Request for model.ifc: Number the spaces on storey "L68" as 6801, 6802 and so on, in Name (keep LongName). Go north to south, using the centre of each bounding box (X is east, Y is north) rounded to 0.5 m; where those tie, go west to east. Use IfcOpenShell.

First a look at what the model holds.

```python
import ifcopenshell
import ifcopenshell.util.element
import ifcopenshell.util.placement

model = ifcopenshell.open("model.ifc")
print(model.schema)
storey = next(s for s in model.by_type("IfcBuildingStorey") if s.Name == "L68")
spaces = [e for e in ifcopenshell.util.element.get_decomposition(storey) if e.is_a("IfcSpace")]
for e in sorted(spaces, key=lambda e: e.id()):
    origin = ifcopenshell.util.placement.get_local_placement(e.ObjectPlacement)[:3, 3]
    print(e.id(), e.Name, e.LongName, origin.round(2) + 0.0, sep=" | ")
```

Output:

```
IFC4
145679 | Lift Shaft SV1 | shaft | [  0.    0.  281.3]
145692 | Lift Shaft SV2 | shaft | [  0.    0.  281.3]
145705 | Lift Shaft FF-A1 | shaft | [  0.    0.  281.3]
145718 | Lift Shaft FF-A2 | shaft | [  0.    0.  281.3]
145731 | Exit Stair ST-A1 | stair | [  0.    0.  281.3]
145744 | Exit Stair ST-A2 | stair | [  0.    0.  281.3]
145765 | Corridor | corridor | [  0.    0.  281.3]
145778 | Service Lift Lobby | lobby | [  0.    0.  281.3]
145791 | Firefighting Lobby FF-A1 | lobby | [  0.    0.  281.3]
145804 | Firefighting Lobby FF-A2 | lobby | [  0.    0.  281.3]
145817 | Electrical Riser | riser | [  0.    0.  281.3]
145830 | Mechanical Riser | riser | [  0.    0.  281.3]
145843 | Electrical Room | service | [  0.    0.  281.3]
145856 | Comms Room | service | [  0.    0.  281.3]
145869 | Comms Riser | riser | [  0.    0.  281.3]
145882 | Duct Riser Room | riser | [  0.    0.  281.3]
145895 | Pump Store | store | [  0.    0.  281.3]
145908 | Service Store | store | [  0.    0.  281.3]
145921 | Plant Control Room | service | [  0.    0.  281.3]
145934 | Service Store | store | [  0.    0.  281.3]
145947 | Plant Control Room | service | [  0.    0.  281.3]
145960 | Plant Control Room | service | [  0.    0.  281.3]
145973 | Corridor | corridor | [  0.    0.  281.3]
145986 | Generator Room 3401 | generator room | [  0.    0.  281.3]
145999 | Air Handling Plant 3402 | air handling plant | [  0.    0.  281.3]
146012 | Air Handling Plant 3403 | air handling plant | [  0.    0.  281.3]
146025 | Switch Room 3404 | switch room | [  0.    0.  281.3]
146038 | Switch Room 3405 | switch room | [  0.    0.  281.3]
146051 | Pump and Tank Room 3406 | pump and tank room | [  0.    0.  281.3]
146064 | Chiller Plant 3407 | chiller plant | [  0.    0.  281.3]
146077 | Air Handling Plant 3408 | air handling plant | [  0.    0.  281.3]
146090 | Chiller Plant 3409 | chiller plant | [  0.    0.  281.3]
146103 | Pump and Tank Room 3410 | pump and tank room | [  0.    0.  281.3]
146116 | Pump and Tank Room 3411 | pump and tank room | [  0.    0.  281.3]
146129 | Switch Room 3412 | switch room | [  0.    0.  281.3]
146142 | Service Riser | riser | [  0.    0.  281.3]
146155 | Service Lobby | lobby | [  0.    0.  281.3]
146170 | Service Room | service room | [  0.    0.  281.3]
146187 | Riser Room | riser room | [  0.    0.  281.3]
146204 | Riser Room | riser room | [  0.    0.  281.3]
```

```python
import ifcopenshell
import ifcopenshell.geom
import ifcopenshell.util.element
import ifcopenshell.util.shape

model = ifcopenshell.open("model.ifc")
settings = ifcopenshell.geom.settings()
settings.set("use-world-coords", True)


def centre(element):
    shape = ifcopenshell.geom.create_shape(settings, element)
    return ifcopenshell.util.shape.get_bbox_centroid(shape.geometry)


storey = next(s for s in model.by_type("IfcBuildingStorey") if s.Name == "L68")
spaces = [e for e in ifcopenshell.util.element.get_decomposition(storey) if e.is_a("IfcSpace")]

# Insertion points can sit at a corner or the storey origin, so sort by the geometry (in metres).
centres = {e: centre(e) for e in spaces}
spaces.sort(key=lambda e: (-round(centres[e][1] / 0.5), centres[e][0]))

for i, e in enumerate(spaces, start=1):
    number = f"68{i:02d}"
    e.Name = number
    print(e.id(), number)

model.write("model_updated.ifc")
```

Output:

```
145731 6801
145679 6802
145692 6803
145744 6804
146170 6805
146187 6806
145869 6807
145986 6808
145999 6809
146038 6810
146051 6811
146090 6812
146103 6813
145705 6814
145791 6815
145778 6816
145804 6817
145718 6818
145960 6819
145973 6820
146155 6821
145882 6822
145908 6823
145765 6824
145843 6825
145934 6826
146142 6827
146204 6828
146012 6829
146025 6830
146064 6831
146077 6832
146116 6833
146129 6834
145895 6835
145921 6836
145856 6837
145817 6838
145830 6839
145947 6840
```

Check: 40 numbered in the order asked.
